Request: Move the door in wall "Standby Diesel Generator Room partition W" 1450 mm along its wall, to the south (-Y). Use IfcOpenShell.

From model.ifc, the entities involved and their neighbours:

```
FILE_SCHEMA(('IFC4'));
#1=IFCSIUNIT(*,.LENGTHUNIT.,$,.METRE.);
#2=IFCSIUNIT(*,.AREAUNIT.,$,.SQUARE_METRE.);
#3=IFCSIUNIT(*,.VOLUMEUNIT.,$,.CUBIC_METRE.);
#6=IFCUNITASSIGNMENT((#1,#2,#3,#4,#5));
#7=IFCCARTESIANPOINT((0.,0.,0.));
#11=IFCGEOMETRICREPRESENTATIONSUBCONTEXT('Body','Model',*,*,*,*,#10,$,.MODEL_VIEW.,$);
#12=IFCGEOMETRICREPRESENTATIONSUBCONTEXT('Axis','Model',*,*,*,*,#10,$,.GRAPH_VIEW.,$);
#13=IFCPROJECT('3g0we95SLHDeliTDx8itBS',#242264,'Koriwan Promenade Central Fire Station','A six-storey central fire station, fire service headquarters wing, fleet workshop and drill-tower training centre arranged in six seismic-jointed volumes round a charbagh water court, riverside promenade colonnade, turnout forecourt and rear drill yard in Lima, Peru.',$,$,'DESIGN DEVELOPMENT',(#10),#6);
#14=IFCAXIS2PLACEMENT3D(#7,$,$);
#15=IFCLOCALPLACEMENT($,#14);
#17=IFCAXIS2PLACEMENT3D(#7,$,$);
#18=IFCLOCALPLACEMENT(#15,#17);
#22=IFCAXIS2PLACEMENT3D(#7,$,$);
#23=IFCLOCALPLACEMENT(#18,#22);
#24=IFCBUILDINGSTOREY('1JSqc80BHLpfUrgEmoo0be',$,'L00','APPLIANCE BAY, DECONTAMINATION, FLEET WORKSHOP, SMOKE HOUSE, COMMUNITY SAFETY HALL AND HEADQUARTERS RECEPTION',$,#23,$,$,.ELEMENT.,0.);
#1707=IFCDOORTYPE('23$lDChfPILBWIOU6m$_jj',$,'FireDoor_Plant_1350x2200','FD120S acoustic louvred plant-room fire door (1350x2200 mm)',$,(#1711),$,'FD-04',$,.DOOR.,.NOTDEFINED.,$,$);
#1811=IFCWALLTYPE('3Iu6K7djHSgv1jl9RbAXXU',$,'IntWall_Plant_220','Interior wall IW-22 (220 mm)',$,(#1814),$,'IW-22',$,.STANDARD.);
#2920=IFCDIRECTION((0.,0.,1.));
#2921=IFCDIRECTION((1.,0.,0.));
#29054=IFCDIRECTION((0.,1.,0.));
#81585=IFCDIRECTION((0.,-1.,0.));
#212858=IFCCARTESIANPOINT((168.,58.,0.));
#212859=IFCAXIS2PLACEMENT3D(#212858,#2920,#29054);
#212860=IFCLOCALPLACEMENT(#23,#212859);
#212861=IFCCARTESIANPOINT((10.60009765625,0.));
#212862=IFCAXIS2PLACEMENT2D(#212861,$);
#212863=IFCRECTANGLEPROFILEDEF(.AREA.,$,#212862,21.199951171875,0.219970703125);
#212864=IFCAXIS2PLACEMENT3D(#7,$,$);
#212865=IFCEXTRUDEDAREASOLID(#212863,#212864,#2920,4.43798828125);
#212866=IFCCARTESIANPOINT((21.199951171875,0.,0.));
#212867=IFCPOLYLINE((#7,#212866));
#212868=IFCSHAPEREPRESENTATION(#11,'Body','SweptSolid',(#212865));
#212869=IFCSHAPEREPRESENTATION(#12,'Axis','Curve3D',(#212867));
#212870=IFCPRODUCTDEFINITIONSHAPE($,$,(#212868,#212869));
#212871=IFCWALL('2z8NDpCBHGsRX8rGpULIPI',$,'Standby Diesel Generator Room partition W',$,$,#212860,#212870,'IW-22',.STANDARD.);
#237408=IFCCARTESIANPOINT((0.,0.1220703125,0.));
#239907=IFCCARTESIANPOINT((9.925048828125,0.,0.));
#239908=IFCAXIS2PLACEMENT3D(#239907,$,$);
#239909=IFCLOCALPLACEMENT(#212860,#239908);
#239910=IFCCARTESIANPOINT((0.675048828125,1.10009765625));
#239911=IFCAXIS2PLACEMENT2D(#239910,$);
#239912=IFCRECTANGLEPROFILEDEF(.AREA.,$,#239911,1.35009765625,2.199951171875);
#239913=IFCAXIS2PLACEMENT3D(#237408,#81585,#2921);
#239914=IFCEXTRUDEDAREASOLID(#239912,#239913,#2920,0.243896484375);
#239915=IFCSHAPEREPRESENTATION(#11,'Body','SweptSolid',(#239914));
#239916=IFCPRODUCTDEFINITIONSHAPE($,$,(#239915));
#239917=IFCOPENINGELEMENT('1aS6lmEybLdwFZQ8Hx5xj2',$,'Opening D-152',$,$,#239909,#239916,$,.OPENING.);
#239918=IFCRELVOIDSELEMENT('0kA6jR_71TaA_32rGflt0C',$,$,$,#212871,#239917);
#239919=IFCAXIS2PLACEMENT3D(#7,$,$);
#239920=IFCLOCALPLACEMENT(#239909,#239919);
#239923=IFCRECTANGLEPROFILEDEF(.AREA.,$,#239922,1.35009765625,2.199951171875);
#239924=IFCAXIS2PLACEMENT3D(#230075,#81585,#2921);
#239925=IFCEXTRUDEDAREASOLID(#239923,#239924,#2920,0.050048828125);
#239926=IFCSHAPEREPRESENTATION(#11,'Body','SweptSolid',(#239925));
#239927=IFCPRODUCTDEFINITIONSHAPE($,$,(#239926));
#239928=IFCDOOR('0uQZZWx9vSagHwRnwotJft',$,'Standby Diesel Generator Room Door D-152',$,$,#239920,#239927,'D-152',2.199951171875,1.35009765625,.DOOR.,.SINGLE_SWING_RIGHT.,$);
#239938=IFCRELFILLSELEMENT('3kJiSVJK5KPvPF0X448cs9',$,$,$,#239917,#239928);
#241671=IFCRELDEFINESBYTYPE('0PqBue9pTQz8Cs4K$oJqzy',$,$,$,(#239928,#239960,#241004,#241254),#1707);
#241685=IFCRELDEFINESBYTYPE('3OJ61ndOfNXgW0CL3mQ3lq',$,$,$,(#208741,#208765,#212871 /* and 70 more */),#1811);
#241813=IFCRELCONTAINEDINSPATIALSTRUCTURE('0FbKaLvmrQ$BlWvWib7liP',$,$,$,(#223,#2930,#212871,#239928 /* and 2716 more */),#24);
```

```python
import ifcopenshell
import ifcopenshell.api.geometry
import ifcopenshell.util.placement
import ifcopenshell.util.unit

model = ifcopenshell.open("model.ifc")
unit_scale = ifcopenshell.util.unit.calculate_unit_scale(model)

door = model.by_guid("0uQZZWx9vSagHwRnwotJft")
opening = door.FillsVoids[0].RelatingOpeningElement
wall = opening.VoidsElements[0].RelatingBuildingElement

wall_matrix = ifcopenshell.util.placement.get_local_placement(wall.ObjectPlacement)
shift = wall_matrix[:3, 0] * -1.45 / unit_scale
before = ifcopenshell.util.placement.get_local_placement(door.ObjectPlacement)[:3, 3].copy()

# The door is placed relative to its opening, so it follows when the opening moves.
matrix = ifcopenshell.util.placement.get_local_placement(opening.ObjectPlacement)
matrix[:3, 3] += shift
ifcopenshell.api.geometry.edit_object_placement(
    model, product=opening, matrix=matrix, is_si=False, should_transform_children=True
)

after = ifcopenshell.util.placement.get_local_placement(door.ObjectPlacement)[:3, 3]
print("door moved by", (after - before).round(3) + 0.0)

model.write("model_edited.ifc")
```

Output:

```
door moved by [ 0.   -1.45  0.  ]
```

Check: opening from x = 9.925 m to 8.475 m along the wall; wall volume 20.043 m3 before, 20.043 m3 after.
